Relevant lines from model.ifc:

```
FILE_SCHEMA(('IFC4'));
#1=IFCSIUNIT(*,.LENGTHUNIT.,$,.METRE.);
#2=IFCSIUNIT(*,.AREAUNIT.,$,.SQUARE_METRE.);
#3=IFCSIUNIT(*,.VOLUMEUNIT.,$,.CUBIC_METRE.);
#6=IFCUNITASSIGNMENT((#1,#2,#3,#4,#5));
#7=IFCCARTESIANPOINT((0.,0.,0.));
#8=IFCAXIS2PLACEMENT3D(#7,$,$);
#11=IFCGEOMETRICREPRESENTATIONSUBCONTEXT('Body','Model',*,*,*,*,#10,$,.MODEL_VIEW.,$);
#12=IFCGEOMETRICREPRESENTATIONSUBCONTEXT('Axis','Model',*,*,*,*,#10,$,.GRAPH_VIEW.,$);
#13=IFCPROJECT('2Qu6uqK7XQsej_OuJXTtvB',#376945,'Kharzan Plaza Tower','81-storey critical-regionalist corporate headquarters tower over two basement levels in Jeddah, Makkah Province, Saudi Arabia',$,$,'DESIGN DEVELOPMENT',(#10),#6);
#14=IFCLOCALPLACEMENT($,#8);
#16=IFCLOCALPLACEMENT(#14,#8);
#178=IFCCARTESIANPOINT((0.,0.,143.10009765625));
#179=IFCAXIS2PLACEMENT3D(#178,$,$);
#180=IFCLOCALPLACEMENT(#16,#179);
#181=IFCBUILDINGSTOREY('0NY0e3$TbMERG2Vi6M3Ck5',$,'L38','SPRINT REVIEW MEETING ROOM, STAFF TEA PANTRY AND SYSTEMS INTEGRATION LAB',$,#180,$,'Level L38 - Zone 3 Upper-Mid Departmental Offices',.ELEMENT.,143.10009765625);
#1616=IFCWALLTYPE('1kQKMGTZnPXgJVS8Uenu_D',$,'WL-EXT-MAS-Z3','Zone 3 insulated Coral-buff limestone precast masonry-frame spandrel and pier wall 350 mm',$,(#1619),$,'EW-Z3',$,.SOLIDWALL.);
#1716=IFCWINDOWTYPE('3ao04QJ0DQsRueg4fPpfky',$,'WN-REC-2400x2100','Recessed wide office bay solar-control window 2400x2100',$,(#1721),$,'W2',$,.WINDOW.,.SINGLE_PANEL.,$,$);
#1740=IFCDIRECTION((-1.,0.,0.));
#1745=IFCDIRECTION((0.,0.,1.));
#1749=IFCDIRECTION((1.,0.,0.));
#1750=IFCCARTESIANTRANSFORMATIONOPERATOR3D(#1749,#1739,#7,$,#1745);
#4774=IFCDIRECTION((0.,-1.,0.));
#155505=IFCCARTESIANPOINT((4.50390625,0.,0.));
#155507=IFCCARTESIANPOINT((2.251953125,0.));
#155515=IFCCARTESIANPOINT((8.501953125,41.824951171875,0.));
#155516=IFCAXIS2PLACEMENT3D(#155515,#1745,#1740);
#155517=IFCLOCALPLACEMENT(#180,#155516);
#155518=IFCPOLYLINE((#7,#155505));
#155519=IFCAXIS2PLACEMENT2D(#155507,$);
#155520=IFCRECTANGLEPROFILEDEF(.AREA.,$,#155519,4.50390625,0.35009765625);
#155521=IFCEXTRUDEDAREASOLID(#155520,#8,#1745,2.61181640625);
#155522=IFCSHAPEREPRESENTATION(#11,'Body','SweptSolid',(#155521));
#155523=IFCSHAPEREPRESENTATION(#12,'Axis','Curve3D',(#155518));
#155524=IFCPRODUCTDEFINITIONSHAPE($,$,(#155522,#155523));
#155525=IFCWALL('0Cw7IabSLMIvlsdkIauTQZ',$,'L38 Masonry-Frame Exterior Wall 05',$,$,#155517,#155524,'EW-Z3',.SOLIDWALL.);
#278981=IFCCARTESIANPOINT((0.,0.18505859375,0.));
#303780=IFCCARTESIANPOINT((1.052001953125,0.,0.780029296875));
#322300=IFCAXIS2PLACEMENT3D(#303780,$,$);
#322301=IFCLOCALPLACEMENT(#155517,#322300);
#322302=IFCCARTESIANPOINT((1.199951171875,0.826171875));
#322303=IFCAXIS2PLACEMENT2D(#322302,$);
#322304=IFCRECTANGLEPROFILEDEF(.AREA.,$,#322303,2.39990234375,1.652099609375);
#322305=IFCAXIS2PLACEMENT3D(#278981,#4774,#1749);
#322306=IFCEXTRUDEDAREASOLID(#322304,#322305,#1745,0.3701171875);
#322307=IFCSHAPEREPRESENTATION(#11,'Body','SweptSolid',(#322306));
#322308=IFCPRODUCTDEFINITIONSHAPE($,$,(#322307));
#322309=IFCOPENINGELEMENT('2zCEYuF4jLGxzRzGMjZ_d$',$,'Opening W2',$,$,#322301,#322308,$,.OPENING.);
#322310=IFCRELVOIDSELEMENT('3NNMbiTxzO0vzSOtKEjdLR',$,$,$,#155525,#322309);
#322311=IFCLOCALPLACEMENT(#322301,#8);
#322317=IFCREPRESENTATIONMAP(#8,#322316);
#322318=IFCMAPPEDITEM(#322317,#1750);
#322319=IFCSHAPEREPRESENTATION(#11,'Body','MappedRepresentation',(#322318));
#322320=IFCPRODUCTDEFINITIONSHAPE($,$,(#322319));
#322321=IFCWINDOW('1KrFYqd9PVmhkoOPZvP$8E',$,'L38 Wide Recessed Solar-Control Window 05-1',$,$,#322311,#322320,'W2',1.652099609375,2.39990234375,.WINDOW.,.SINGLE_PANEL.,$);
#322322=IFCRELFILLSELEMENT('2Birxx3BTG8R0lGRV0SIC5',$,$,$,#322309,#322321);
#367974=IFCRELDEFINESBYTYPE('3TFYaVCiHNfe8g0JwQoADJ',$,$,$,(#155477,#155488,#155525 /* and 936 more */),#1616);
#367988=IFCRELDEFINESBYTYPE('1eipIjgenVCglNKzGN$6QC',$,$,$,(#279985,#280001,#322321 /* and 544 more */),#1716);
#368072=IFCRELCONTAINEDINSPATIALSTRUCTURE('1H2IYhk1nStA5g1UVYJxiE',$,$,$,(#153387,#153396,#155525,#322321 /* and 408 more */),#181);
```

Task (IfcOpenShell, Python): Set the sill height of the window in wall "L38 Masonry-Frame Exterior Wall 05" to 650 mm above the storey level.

```python
import numpy as np
import ifcopenshell
import ifcopenshell.api.geometry
import ifcopenshell.geom
import ifcopenshell.util.element
import ifcopenshell.util.placement
import ifcopenshell.util.shape
import ifcopenshell.util.unit

model = ifcopenshell.open("model.ifc")
unit_scale = ifcopenshell.util.unit.calculate_unit_scale(model)

window = model.by_guid("1KrFYqd9PVmhkoOPZvP$8E")
opening = window.FillsVoids[0].RelatingOpeningElement
storey = ifcopenshell.util.element.get_container(window, ifc_class="IfcBuildingStorey")
level = ifcopenshell.util.placement.get_local_placement(storey.ObjectPlacement)[2, 3]

# The opening's origin need not be at the sill, so measure its lowest point.
shape = ifcopenshell.geom.create_shape(ifcopenshell.geom.settings(), opening)
bottom = ifcopenshell.util.shape.get_shape_bottom_elevation(shape, shape.geometry) / unit_scale
dz = level + 0.65 - bottom

shift = np.array([0.0, 0.0, dz])
# The window is placed relative to its opening, so it follows when the opening moves.
matrix = ifcopenshell.util.placement.get_local_placement(opening.ObjectPlacement)
matrix[:3, 3] += shift
ifcopenshell.api.geometry.edit_object_placement(
    model, product=opening, matrix=matrix, is_si=False, should_transform_children=True
)

print(f"moved by {dz * unit_scale:+.3f} m")

model.write("model-out.ifc")
```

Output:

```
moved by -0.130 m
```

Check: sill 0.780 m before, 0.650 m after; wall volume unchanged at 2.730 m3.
